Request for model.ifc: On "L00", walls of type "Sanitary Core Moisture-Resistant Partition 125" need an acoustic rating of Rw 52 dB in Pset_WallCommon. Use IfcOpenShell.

First a look at what the model holds.

```python
import ifcopenshell
import ifcopenshell.util.element

model = ifcopenshell.open("model.ifc")
print(model.schema)
storey = next(s for s in model.by_type("IfcBuildingStorey") if s.Name == "L00")
walls = [e for e in ifcopenshell.util.element.get_decomposition(storey) if e.is_a("IfcWall")]
seen = {}
for e in walls:
    element_type = ifcopenshell.util.element.get_type(e)
    key = (element_type.Name if element_type != e and element_type else None, ifcopenshell.util.element.get_pset(e, "Pset_WallCommon", "AcousticRating"))
    seen[key] = seen.get(key, 0) + 1
for (name, value), count in sorted(seen.items(), key=str):
    print(count, "x", name, "|", value)
```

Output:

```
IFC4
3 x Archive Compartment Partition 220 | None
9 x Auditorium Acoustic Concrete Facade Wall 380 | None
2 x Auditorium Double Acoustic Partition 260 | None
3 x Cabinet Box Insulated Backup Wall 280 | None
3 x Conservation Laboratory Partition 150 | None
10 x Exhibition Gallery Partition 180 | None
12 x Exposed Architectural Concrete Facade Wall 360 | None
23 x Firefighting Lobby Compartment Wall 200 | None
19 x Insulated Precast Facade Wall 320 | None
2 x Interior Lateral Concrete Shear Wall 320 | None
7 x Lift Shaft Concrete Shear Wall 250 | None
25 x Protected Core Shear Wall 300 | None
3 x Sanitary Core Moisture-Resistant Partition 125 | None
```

```python
import ifcopenshell
import ifcopenshell.api.pset
import ifcopenshell.util.element

model = ifcopenshell.open("model.ifc")

storey = next(s for s in model.by_type("IfcBuildingStorey") if s.Name == "L00")
walls = [e for e in ifcopenshell.util.element.get_decomposition(storey) if e.is_a("IfcWall")]

count = 0
for e in walls:
    element_type = ifcopenshell.util.element.get_type(e)
    if element_type in (None, e) or element_type.Name != "Sanitary Core Moisture-Resistant Partition 125":
        continue
    # add_pset returns the element's existing set when there is one.
    pset = ifcopenshell.api.pset.add_pset(model, product=e, name="Pset_WallCommon")
    ifcopenshell.api.pset.edit_pset(model, pset=pset, properties={"AcousticRating": "Rw 52 dB"})
    count += 1

print(count, "walls updated")

model.write("model_updated.ifc")
```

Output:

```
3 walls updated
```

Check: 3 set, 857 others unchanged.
